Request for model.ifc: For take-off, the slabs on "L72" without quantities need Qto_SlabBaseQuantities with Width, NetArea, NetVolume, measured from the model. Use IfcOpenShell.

First a look at what the model holds.

```python
import ifcopenshell
import ifcopenshell.util.element
import ifcopenshell.util.unit

model = ifcopenshell.open("model.ifc")
print(model.schema)
for unit_type in ("LENGTHUNIT", "AREAUNIT", "VOLUMEUNIT"):
    print(unit_type, ifcopenshell.util.unit.calculate_unit_scale(model, unit_type))
storey = next(s for s in model.by_type("IfcBuildingStorey") if s.Name == "L72")
slabs = [e for e in ifcopenshell.util.element.get_decomposition(storey) if e.is_a("IfcSlab")]
for e in sorted(slabs, key=lambda e: e.id()):
    print(e.id(), e.is_a(), e.Name, list(ifcopenshell.util.element.get_psets(e, qtos_only=True)), sep=" | ")
```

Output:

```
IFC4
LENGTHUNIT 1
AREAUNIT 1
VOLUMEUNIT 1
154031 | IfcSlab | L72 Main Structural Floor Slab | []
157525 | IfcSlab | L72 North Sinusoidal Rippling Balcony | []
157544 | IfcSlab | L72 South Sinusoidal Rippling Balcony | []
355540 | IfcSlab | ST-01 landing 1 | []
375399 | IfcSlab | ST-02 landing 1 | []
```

```python
import ifcopenshell
import ifcopenshell.api.pset
import ifcopenshell.geom
import ifcopenshell.util.element
import ifcopenshell.util.shape
import ifcopenshell.util.unit

model = ifcopenshell.open("model.ifc")
unit_scale = ifcopenshell.util.unit.calculate_unit_scale(model)
area_scale = ifcopenshell.util.unit.calculate_unit_scale(model, "AREAUNIT")
volume_scale = ifcopenshell.util.unit.calculate_unit_scale(model, "VOLUMEUNIT")
settings = ifcopenshell.geom.settings()

storey = next(s for s in model.by_type("IfcBuildingStorey") if s.Name == "L72")
slabs = [e for e in ifcopenshell.util.element.get_decomposition(storey) if e.is_a("IfcSlab")]

for e in sorted(slabs, key=lambda e: e.id()):
    if ifcopenshell.util.element.get_psets(e, qtos_only=True, should_inherit=False):
        continue
    # Geometry comes back in metres, in the element's own axes.
    shape = ifcopenshell.geom.create_shape(settings, e)
    values = {
        "Width": ifcopenshell.util.shape.get_z(shape.geometry) / unit_scale,
        "NetArea": ifcopenshell.util.shape.get_footprint_area(shape.geometry) / area_scale,
        "NetVolume": ifcopenshell.util.shape.get_volume(shape.geometry) / volume_scale,
    }
    qto = ifcopenshell.api.pset.add_qto(model, product=e, name="Qto_SlabBaseQuantities")
    ifcopenshell.api.pset.edit_qto(model, qto=qto, properties=values)
    print(e.id(), {k: round(v, 3) for k, v in values.items()})

model.write("model-out.ifc")
```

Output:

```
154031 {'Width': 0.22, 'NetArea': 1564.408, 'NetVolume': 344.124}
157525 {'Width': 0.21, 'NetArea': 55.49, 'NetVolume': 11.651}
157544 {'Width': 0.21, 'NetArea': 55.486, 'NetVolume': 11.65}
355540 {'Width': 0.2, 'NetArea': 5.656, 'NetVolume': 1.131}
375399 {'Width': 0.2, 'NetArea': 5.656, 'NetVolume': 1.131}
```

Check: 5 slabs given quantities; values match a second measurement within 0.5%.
